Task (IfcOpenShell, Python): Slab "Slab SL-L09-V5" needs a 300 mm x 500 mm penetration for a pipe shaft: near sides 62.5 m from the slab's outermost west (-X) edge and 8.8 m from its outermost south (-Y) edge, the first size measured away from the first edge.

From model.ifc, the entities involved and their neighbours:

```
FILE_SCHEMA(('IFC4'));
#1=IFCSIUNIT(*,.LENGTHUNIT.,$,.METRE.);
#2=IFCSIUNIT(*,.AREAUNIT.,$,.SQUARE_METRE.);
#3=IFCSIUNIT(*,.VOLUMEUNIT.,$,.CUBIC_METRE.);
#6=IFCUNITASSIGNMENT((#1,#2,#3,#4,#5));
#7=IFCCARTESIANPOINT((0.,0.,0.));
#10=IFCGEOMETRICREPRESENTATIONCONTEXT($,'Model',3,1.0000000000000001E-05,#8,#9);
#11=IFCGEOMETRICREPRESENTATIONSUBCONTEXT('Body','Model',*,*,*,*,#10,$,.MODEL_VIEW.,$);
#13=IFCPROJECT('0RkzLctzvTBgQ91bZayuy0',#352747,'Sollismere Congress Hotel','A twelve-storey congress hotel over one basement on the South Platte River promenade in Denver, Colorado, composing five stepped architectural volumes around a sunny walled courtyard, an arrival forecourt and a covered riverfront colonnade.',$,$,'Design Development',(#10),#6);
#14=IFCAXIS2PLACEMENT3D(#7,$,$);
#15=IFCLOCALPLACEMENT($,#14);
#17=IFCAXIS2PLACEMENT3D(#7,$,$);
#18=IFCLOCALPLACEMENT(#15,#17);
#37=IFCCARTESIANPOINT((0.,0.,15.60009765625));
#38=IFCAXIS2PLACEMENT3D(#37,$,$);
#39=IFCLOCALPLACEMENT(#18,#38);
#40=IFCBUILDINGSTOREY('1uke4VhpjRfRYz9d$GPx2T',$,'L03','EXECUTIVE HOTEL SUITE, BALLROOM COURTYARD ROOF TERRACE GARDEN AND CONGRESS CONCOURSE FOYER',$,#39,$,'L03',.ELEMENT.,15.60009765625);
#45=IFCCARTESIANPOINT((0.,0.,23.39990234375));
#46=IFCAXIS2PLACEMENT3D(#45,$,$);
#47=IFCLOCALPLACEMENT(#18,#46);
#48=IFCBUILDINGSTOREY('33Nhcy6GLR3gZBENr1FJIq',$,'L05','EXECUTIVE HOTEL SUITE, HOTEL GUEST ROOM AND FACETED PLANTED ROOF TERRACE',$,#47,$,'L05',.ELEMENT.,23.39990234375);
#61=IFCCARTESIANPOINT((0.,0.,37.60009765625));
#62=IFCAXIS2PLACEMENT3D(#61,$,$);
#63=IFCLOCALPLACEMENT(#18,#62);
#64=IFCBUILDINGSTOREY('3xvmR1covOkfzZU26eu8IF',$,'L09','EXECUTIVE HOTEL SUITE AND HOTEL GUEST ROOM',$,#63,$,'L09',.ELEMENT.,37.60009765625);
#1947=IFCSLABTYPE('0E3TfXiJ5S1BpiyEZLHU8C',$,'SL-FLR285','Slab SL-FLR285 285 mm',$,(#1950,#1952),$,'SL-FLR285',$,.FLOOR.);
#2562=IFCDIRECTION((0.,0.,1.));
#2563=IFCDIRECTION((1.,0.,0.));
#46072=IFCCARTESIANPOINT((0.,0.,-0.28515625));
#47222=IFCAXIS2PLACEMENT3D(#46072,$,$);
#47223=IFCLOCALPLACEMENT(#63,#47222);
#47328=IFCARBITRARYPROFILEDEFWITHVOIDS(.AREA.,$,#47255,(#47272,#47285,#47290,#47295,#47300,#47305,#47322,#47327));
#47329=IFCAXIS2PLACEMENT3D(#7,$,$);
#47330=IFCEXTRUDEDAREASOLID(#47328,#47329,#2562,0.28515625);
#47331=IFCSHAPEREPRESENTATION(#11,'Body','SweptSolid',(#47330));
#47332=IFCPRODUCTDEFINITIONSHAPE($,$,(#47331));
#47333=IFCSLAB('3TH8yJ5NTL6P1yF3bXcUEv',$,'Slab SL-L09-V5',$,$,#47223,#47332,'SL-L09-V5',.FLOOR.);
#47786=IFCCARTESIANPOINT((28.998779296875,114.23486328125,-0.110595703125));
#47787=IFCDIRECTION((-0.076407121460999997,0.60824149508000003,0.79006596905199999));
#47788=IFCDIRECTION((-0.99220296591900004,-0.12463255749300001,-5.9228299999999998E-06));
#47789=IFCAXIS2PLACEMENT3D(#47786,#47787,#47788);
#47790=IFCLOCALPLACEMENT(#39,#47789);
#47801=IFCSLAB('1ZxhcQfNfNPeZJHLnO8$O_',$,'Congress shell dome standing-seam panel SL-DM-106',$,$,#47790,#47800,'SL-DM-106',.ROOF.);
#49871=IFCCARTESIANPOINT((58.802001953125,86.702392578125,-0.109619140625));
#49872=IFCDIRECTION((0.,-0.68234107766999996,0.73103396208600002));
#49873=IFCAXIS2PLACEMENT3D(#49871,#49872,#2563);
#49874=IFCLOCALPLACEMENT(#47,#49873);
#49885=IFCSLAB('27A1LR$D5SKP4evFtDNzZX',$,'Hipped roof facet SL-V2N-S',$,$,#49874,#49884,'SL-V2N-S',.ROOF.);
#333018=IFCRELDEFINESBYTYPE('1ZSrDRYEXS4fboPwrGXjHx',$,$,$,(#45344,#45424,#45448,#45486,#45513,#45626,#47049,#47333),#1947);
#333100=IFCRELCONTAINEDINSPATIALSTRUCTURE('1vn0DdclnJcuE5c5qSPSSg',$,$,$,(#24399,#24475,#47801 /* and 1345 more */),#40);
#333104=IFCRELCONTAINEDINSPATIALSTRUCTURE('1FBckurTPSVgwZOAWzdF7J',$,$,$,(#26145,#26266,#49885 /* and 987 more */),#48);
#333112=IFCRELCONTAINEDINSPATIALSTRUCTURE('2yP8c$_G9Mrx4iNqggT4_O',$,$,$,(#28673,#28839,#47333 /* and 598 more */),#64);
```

```python
import numpy as np
import ifcopenshell
import ifcopenshell.api.feature
import ifcopenshell.api.geometry
import ifcopenshell.api.root
import ifcopenshell.geom
import ifcopenshell.util.placement
import ifcopenshell.util.representation
import ifcopenshell.util.shape
import ifcopenshell.util.unit

model = ifcopenshell.open("model.ifc")
unit_scale = ifcopenshell.util.unit.calculate_unit_scale(model)
settings = ifcopenshell.geom.settings()


def volume(element):
    """Net volume in cubic metres, openings subtracted."""
    shape = ifcopenshell.geom.create_shape(settings, element)
    return ifcopenshell.util.shape.get_volume(shape.geometry)


slab = model.by_id(47333)
before = volume(slab)

# Extent in the slab's own axes, in metres. The edges named are its -X and -Y sides.
slab_shape = ifcopenshell.geom.create_shape(settings, slab)
vertices = ifcopenshell.util.shape.get_vertices(slab_shape.geometry)
x_min, y_min, bottom = vertices.min(axis=0)
top = vertices[:, 2].max()

opening = ifcopenshell.api.root.create_entity(model, ifc_class="IfcOpeningElement", name="Pipe shaft opening", predefined_type="OPENING")
context = ifcopenshell.util.representation.get_context(model, "Model", "Body", "MODEL_VIEW")
width, depth = 0.3, 0.5
outline = [(0.0, 0.0), (width, 0.0), (width, depth), (0.0, depth), (0.0, 0.0)]
# Overshoot both faces by 50 mm so the cut is clean.
shape = ifcopenshell.api.geometry.add_slab_representation(
    model, context=context, depth=top - bottom + 0.1, polyline=outline
)
ifcopenshell.api.geometry.assign_representation(model, product=opening, representation=shape)

matrix = ifcopenshell.util.placement.get_local_placement(slab.ObjectPlacement)
matrix[:, 3] = matrix @ np.append(np.array([x_min + 62.5, y_min + 8.8, bottom - 0.05]) / unit_scale, 1.0)
ifcopenshell.api.geometry.edit_object_placement(model, product=opening, matrix=matrix, is_si=False)
ifcopenshell.api.feature.add_feature(model, feature=opening, element=slab)

after = volume(slab)

print(f"slab volume {before:.3f} -> {after:.3f} m3")

model.write("model_edited.ifc")
```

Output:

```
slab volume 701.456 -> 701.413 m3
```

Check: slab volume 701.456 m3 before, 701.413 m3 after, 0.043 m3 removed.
